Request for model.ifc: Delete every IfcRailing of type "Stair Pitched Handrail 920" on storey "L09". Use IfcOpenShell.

First a look at what the model holds.

```python
import ifcopenshell
import ifcopenshell.util.element

model = ifcopenshell.open("model.ifc")
print(model.schema)
storey = next(s for s in model.by_type("IfcBuildingStorey") if s.Name == "L09")
railings = [e for e in ifcopenshell.util.element.get_decomposition(storey) if e.is_a("IfcRailing")]
seen = {}
for e in railings:
    element_type = ifcopenshell.util.element.get_type(e)
    name = element_type.Name if element_type not in (None, e) else None
    seen[name] = seen.get(name, 0) + 1
for name, count in sorted(seen.items(), key=str):
    print(count, "x", name)
```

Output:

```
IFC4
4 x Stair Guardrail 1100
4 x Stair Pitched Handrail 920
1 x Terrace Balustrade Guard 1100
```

```python
import ifcopenshell
import ifcopenshell.api.root
import ifcopenshell.util.element

model = ifcopenshell.open("model.ifc")

storey = next(s for s in model.by_type("IfcBuildingStorey") if s.Name == "L09")
railings = [e for e in ifcopenshell.util.element.get_decomposition(storey) if e.is_a("IfcRailing")]
targets = [e for e in railings if (t := ifcopenshell.util.element.get_type(e)) not in (None, e) and t.Name == "Stair Pitched Handrail 920"]

for e in targets:
    ifcopenshell.api.root.remove_product(model, product=e)
print(len(targets), "removed")

model.write("model_rev.ifc")
```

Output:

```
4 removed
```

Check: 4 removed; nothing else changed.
